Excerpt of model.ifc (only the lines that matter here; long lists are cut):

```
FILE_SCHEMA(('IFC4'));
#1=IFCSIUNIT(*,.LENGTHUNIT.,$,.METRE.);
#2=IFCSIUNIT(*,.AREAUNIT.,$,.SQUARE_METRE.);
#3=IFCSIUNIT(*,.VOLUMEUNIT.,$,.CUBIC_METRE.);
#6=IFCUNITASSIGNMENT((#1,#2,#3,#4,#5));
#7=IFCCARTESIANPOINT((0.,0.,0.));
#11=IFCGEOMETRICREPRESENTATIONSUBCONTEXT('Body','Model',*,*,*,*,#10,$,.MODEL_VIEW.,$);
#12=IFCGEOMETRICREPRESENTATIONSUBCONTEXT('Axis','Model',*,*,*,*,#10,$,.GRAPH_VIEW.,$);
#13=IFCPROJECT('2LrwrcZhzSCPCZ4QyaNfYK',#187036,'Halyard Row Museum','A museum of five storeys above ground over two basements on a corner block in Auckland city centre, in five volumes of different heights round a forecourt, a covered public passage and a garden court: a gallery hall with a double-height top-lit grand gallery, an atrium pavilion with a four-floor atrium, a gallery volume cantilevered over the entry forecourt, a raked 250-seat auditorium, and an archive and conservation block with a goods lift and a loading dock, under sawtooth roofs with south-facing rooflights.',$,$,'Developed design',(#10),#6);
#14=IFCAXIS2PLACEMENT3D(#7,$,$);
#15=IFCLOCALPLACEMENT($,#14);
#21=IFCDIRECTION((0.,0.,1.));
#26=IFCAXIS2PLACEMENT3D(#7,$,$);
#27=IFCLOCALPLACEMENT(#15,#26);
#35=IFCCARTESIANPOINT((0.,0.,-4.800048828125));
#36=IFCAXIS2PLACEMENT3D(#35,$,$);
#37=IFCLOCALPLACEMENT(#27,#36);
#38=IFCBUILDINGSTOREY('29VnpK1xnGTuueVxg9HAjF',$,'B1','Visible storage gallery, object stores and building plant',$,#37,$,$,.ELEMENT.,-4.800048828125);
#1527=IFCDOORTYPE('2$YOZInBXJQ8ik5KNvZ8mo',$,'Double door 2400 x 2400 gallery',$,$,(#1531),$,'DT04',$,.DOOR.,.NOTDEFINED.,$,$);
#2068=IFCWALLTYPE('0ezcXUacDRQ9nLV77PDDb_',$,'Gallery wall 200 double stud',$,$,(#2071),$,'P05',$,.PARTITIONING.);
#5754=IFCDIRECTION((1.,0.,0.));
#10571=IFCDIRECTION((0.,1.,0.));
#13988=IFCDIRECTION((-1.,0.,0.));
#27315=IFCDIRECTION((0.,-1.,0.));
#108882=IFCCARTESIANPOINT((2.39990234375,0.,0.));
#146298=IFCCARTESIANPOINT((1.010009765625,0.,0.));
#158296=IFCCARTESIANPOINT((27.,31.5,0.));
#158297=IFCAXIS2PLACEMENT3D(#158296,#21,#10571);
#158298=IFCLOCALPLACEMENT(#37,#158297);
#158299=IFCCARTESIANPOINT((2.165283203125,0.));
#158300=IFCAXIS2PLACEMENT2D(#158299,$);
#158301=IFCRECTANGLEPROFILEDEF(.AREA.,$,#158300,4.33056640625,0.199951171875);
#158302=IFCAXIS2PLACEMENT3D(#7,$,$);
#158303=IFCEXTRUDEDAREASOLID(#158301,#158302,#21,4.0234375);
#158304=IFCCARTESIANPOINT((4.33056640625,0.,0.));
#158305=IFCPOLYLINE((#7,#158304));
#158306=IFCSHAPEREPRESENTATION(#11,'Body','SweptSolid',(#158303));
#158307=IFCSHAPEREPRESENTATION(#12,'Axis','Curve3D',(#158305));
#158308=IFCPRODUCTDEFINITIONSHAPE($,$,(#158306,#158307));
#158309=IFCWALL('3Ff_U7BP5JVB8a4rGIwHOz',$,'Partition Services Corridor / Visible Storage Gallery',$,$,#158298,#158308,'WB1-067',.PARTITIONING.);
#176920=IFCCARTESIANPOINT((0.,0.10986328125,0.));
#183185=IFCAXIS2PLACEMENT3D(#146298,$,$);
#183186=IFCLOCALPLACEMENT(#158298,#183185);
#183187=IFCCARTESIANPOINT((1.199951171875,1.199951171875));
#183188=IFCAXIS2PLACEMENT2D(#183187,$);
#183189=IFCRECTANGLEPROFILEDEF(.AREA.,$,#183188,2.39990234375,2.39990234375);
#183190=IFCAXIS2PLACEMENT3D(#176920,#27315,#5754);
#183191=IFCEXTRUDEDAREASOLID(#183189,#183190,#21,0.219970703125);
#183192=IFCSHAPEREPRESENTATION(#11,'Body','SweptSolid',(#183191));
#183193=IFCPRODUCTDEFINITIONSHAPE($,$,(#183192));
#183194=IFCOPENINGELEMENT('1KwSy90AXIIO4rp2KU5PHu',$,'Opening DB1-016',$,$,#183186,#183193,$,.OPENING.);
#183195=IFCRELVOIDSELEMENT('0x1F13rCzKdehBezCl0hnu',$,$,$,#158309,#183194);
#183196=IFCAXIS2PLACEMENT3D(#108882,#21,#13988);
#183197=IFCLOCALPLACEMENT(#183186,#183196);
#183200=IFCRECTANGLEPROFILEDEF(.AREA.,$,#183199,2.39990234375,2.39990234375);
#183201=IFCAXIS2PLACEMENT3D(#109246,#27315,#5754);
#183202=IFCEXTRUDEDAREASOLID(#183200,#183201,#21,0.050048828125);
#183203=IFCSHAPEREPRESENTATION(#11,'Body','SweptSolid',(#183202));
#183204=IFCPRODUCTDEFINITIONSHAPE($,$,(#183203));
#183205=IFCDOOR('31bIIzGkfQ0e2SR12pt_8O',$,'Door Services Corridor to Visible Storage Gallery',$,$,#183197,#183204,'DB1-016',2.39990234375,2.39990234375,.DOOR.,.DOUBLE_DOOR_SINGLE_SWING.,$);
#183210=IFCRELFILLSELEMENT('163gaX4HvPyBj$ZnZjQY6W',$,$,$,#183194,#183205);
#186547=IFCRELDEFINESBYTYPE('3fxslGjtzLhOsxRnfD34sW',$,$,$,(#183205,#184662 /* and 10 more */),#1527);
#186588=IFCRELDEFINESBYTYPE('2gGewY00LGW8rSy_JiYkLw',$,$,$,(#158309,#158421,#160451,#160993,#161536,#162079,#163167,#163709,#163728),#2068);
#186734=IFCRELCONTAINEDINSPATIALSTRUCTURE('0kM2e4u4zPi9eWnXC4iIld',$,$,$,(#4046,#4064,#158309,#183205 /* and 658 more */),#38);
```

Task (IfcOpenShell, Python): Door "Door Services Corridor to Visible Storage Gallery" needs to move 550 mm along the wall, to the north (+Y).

```python
import ifcopenshell
import ifcopenshell.api.geometry
import ifcopenshell.util.placement
import ifcopenshell.util.unit

model = ifcopenshell.open("model.ifc")
unit_scale = ifcopenshell.util.unit.calculate_unit_scale(model)

door = model.by_guid("31bIIzGkfQ0e2SR12pt_8O")
opening = door.FillsVoids[0].RelatingOpeningElement
wall = opening.VoidsElements[0].RelatingBuildingElement

wall_matrix = ifcopenshell.util.placement.get_local_placement(wall.ObjectPlacement)
shift = wall_matrix[:3, 0] * 0.55 / unit_scale
before = ifcopenshell.util.placement.get_local_placement(door.ObjectPlacement)[:3, 3].copy()

# The door is placed relative to its opening, so it follows when the opening moves.
matrix = ifcopenshell.util.placement.get_local_placement(opening.ObjectPlacement)
matrix[:3, 3] += shift
ifcopenshell.api.geometry.edit_object_placement(
    model, product=opening, matrix=matrix, is_si=False, should_transform_children=True
)

after = ifcopenshell.util.placement.get_local_placement(door.ObjectPlacement)[:3, 3]
print("door moved by", (after - before).round(3) + 0.0)

model.write("model_v2.ifc")
```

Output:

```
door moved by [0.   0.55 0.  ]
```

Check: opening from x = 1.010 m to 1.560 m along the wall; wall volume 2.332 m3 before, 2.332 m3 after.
